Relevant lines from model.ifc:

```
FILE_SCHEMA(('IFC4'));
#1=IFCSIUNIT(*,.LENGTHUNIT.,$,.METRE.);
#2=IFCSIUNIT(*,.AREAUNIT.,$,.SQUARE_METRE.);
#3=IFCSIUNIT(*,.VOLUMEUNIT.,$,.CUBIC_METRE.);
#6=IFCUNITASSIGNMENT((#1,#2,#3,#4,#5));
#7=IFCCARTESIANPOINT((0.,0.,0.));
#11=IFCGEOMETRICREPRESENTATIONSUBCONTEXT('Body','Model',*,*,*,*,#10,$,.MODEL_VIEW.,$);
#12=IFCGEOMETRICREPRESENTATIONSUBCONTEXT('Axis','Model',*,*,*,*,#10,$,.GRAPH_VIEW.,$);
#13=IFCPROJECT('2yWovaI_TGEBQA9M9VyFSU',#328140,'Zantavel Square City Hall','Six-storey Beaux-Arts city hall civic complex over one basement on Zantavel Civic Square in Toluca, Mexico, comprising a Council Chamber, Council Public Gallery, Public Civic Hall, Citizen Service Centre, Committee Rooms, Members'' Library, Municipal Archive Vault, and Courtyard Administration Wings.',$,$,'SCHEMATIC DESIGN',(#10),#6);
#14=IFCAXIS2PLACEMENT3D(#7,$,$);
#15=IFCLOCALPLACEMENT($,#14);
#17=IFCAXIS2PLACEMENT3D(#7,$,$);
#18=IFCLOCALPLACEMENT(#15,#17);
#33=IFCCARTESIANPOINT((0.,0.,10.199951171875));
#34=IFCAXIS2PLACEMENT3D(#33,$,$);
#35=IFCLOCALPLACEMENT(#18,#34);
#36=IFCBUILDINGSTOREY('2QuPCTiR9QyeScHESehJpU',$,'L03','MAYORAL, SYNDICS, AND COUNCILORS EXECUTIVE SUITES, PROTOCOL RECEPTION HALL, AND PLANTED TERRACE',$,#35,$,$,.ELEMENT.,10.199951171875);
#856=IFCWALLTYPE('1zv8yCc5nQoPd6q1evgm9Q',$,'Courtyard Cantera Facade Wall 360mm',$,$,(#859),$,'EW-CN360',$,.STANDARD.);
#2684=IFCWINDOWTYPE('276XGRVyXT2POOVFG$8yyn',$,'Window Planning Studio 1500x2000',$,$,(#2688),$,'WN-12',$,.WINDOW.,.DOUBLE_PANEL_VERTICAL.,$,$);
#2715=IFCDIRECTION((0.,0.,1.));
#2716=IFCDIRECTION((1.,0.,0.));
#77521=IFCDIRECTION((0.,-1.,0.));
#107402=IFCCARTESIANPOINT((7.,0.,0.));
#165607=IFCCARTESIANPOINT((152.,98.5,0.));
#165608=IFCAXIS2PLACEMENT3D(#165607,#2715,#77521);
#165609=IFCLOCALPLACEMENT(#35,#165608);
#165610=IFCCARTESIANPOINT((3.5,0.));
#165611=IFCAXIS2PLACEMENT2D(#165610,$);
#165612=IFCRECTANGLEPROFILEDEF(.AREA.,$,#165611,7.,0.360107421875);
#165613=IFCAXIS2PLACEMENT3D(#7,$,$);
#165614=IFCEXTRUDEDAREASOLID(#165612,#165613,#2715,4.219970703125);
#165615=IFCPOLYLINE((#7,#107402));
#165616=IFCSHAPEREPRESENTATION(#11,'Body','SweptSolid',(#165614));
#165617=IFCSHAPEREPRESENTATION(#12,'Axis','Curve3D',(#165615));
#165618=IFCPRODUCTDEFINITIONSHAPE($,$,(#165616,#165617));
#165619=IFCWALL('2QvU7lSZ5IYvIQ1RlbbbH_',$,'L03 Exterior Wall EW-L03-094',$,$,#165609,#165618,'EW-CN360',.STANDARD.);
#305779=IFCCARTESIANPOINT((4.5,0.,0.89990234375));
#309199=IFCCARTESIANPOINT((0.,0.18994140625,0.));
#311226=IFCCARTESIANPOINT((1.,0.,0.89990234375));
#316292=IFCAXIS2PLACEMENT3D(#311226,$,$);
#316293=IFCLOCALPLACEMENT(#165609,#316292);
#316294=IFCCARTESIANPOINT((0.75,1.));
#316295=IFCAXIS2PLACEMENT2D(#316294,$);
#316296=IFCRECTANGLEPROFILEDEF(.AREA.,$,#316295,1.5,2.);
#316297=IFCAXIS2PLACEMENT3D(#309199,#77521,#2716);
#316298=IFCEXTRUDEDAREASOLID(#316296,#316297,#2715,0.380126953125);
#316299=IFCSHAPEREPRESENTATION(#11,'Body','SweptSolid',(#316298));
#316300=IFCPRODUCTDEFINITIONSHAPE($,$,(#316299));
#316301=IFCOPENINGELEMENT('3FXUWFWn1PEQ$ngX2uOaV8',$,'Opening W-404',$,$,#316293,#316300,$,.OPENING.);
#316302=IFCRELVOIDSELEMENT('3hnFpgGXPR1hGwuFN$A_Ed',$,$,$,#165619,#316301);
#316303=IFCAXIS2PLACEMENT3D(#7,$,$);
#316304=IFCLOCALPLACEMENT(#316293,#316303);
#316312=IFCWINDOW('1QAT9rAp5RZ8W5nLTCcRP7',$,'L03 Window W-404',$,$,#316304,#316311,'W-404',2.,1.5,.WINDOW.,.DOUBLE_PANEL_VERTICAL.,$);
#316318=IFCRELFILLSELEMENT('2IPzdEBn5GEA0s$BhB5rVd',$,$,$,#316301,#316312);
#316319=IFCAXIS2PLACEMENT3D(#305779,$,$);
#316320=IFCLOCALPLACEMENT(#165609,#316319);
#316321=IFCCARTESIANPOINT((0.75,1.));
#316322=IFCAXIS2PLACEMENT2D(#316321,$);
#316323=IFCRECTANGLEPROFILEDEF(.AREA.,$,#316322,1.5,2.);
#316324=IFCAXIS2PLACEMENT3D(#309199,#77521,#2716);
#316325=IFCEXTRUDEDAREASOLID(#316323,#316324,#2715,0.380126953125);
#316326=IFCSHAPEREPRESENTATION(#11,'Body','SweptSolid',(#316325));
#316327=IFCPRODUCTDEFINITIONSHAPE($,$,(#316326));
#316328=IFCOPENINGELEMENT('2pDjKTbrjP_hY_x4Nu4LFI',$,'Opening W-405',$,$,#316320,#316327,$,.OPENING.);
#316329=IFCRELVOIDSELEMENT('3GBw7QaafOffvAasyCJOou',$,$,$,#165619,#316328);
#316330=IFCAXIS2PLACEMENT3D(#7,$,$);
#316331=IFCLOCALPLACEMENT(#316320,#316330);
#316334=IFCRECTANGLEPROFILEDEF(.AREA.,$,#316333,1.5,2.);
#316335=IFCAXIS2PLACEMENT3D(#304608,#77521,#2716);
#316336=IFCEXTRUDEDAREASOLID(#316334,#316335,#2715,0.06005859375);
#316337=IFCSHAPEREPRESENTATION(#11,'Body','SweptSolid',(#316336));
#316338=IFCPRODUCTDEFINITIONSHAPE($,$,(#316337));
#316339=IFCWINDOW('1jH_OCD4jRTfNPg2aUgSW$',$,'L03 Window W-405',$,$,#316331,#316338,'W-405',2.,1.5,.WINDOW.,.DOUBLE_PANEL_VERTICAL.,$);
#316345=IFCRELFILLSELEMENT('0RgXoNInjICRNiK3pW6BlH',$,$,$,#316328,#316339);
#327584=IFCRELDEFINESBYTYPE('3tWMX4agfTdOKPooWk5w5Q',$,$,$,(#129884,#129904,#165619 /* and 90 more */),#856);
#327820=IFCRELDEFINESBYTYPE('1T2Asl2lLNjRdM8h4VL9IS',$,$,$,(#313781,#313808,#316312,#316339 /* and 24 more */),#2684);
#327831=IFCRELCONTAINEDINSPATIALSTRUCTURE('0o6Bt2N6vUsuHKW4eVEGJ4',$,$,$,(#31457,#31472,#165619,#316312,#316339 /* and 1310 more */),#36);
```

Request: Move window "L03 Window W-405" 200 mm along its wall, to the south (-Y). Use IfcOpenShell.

```python
import ifcopenshell
import ifcopenshell.api.geometry
import ifcopenshell.util.placement
import ifcopenshell.util.unit

model = ifcopenshell.open("model.ifc")
unit_scale = ifcopenshell.util.unit.calculate_unit_scale(model)

window = model.by_guid("1jH_OCD4jRTfNPg2aUgSW$")
opening = window.FillsVoids[0].RelatingOpeningElement
wall = opening.VoidsElements[0].RelatingBuildingElement

wall_matrix = ifcopenshell.util.placement.get_local_placement(wall.ObjectPlacement)
shift = wall_matrix[:3, 0] * 0.2 / unit_scale
before = ifcopenshell.util.placement.get_local_placement(window.ObjectPlacement)[:3, 3].copy()

# The window is placed relative to its opening, so it follows when the opening moves.
matrix = ifcopenshell.util.placement.get_local_placement(opening.ObjectPlacement)
matrix[:3, 3] += shift
ifcopenshell.api.geometry.edit_object_placement(
    model, product=opening, matrix=matrix, is_si=False, should_transform_children=True
)

after = ifcopenshell.util.placement.get_local_placement(window.ObjectPlacement)[:3, 3]
print("window moved by", (after - before).round(3) + 0.0)

model.write("model_edited.ifc")
```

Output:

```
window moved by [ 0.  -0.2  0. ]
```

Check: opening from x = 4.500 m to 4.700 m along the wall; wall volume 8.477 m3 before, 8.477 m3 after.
